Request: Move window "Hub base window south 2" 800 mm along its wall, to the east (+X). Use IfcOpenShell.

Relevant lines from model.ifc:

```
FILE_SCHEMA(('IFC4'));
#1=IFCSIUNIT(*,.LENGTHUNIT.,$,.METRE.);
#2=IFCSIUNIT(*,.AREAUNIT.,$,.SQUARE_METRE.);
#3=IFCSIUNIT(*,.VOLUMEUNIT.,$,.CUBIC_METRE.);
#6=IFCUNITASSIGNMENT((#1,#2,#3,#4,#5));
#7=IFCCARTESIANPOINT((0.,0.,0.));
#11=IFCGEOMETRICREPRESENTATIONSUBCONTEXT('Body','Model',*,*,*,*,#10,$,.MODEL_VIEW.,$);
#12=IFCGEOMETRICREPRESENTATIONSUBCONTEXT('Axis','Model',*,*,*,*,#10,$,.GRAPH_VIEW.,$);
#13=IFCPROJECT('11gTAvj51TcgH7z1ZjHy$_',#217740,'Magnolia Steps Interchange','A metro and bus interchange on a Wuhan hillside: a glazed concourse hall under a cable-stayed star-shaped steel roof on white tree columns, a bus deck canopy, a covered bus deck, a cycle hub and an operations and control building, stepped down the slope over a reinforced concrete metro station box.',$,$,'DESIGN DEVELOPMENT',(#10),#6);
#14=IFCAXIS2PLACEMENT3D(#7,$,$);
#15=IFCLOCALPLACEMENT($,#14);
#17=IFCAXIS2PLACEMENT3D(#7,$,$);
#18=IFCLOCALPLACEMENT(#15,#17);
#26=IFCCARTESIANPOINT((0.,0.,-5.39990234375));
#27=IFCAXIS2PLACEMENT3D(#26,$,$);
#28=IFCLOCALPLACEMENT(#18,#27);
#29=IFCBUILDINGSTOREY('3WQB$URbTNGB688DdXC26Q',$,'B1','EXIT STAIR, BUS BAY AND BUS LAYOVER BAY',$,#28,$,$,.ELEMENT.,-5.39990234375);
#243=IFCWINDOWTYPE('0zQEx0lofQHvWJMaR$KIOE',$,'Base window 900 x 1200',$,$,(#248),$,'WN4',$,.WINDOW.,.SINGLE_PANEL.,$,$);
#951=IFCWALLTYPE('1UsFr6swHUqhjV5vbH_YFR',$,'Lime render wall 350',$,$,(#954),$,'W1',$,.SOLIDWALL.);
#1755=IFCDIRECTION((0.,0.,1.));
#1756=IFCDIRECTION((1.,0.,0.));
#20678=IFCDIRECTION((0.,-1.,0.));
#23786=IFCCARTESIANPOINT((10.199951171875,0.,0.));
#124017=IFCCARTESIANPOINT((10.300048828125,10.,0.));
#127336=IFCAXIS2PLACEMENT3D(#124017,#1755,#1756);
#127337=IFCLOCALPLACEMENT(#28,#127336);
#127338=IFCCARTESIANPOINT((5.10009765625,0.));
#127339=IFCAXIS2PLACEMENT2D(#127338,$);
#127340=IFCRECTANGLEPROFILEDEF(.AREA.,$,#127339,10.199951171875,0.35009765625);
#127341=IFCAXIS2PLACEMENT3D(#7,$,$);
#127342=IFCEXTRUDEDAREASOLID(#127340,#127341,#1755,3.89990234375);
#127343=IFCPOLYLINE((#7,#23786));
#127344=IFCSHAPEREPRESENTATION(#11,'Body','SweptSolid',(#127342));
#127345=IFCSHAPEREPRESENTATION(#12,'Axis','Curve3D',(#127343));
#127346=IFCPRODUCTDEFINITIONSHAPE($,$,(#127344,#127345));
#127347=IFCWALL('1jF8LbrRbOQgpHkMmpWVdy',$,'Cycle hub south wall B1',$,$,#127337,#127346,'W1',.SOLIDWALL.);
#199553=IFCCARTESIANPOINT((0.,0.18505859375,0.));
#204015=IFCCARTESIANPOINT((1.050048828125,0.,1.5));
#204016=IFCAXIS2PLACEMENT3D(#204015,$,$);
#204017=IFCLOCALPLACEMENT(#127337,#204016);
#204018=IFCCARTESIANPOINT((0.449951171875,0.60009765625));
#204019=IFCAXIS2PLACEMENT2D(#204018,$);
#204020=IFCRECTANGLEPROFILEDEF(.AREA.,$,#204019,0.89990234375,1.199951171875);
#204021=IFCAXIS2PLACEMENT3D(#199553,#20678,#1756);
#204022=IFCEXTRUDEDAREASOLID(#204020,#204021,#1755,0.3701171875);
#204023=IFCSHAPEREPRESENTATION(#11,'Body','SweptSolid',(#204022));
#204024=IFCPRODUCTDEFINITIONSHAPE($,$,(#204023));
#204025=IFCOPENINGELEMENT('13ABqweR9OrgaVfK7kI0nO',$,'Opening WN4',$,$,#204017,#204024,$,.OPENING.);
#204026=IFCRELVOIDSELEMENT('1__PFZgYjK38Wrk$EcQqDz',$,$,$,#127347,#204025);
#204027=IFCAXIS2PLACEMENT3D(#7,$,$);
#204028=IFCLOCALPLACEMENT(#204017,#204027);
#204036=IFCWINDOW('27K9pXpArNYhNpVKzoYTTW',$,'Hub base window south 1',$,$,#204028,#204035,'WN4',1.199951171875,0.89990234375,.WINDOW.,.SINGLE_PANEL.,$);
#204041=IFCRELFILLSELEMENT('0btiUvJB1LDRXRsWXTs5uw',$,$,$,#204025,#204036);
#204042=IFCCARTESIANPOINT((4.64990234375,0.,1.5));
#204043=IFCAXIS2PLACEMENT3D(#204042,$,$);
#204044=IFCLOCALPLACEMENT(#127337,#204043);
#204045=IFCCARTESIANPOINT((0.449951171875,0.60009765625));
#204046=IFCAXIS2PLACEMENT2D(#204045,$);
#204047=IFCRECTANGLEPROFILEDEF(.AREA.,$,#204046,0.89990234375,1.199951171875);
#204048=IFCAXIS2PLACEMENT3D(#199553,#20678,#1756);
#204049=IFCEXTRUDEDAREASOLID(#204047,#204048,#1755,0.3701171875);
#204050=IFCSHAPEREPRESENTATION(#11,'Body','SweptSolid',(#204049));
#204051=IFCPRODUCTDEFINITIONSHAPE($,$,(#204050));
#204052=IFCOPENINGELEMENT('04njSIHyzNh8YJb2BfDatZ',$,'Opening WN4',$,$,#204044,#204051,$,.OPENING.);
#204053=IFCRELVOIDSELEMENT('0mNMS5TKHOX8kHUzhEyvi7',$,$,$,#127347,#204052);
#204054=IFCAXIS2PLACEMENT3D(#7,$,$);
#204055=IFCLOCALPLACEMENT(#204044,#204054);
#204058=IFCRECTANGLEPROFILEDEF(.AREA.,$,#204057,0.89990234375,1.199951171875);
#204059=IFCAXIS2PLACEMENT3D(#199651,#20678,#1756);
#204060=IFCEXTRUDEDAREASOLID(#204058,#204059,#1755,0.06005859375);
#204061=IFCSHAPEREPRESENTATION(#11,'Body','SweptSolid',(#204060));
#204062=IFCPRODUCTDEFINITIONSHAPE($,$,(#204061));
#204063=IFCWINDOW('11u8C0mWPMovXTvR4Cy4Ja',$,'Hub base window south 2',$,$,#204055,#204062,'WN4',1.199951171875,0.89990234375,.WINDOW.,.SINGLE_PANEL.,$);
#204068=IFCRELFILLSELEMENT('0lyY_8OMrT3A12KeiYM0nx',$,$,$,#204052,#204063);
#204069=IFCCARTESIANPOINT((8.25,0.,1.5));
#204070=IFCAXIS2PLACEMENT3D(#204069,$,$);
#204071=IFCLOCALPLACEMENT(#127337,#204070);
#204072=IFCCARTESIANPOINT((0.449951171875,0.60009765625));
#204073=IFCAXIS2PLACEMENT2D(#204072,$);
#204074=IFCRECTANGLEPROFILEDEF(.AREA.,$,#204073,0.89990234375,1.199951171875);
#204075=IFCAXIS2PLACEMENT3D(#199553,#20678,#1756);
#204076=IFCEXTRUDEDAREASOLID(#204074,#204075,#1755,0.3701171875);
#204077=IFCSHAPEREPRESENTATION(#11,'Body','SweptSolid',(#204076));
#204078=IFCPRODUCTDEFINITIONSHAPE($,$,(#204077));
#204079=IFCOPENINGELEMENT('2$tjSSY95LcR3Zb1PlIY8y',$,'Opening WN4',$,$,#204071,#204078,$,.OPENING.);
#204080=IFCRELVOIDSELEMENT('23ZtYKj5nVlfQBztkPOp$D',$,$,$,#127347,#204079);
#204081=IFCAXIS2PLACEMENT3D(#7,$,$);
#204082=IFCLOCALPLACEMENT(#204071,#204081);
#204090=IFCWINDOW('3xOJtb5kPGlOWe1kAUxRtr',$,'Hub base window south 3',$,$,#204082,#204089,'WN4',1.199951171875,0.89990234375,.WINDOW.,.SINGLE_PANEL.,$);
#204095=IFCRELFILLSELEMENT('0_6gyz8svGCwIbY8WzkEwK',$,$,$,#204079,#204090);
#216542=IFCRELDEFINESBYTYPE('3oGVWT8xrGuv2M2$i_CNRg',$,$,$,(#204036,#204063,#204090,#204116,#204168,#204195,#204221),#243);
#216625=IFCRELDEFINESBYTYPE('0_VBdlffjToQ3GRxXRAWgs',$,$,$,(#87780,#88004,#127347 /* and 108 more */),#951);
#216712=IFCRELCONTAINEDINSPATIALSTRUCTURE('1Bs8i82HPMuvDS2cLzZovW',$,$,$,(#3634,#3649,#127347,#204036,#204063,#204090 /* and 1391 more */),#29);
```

```python
import ifcopenshell
import ifcopenshell.api.geometry
import ifcopenshell.util.placement

model = ifcopenshell.open("model.ifc")

window = model.by_guid("11u8C0mWPMovXTvR4Cy4Ja")
opening = window.FillsVoids[0].RelatingOpeningElement
wall = opening.VoidsElements[0].RelatingBuildingElement

wall_matrix = ifcopenshell.util.placement.get_local_placement(wall.ObjectPlacement)
shift = wall_matrix[:3, 0] * 0.8
before = ifcopenshell.util.placement.get_local_placement(window.ObjectPlacement)[:3, 3].copy()

# The window is placed relative to its opening, so it follows when the opening moves.
matrix = ifcopenshell.util.placement.get_local_placement(opening.ObjectPlacement)
matrix[:3, 3] += shift
ifcopenshell.api.geometry.edit_object_placement(
    model, product=opening, matrix=matrix, is_si=False, should_transform_children=True
)

after = ifcopenshell.util.placement.get_local_placement(window.ObjectPlacement)[:3, 3]
print("window moved by", (after - before).round(3) + 0.0)

model.write("model-out.ifc")
```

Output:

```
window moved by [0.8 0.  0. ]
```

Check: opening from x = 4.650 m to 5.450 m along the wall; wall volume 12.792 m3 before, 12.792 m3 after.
